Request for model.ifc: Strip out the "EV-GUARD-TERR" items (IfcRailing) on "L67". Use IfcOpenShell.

First a look at what the model holds.

```python
import ifcopenshell
import ifcopenshell.util.element

model = ifcopenshell.open("model.ifc")
print(model.schema)
storey = next(s for s in model.by_type("IfcBuildingStorey") if s.Name == "L67")
railings = [e for e in ifcopenshell.util.element.get_decomposition(storey) if e.is_a("IfcRailing")]
seen = {}
for e in railings:
    element_type = ifcopenshell.util.element.get_type(e)
    name = element_type.Name if element_type not in (None, e) else None
    seen[name] = seen.get(name, 0) + 1
for name, count in sorted(seen.items(), key=str):
    print(count, "x", name)
```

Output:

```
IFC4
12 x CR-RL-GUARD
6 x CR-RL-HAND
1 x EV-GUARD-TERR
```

```python
import ifcopenshell
import ifcopenshell.api.root
import ifcopenshell.util.element

model = ifcopenshell.open("model.ifc")

storey = next(s for s in model.by_type("IfcBuildingStorey") if s.Name == "L67")
railings = [e for e in ifcopenshell.util.element.get_decomposition(storey) if e.is_a("IfcRailing")]
targets = [e for e in railings if (t := ifcopenshell.util.element.get_type(e)) not in (None, e) and t.Name == "EV-GUARD-TERR"]

for e in targets:
    ifcopenshell.api.root.remove_product(model, product=e)
print(len(targets), "removed")

model.write("model_edited.ifc")
```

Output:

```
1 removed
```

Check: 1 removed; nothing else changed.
